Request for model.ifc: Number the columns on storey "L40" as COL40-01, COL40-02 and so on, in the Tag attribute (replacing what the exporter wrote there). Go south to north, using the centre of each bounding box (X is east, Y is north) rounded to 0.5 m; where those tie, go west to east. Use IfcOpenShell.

First a look at what the model holds.

```python
import ifcopenshell
import ifcopenshell.util.element
import ifcopenshell.util.placement

model = ifcopenshell.open("model.ifc")
print(model.schema)
storey = next(s for s in model.by_type("IfcBuildingStorey") if s.Name == "L40")
columns = [e for e in ifcopenshell.util.element.get_decomposition(storey) if e.is_a("IfcColumn")]
for e in sorted(columns, key=lambda e: e.id()):
    origin = ifcopenshell.util.placement.get_local_placement(e.ObjectPlacement)[:3, 3]
    print(e.id(), e.Tag, e.Name, origin.round(2) + 0.0, sep=" | ")
```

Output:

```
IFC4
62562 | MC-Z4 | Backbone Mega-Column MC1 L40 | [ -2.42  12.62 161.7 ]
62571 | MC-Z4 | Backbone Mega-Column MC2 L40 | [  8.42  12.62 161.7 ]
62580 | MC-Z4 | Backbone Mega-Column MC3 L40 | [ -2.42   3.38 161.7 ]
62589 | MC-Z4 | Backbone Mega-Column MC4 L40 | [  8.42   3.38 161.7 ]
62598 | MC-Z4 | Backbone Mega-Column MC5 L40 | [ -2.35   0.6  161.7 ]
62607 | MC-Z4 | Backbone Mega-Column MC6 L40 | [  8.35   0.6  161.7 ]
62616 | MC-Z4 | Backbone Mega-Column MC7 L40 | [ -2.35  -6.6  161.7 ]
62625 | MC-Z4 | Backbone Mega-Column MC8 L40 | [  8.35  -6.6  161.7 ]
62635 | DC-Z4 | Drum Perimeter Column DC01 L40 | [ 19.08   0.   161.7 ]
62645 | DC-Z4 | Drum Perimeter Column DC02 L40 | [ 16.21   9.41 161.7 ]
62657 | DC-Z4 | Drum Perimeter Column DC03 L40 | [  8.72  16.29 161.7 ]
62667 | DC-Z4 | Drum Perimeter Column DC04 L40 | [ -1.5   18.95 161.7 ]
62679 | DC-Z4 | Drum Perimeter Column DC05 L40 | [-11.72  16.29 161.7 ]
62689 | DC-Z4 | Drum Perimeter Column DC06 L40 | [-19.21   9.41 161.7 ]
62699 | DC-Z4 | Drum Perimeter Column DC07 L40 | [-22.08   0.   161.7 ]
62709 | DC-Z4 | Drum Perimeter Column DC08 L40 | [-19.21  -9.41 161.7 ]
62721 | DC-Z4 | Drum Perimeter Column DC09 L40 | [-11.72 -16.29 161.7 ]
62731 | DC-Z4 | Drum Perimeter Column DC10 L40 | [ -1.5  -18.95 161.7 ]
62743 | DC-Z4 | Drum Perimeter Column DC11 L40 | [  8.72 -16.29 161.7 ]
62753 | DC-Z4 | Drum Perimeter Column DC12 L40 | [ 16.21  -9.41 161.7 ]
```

```python
import ifcopenshell
import ifcopenshell.geom
import ifcopenshell.util.element
import ifcopenshell.util.shape

model = ifcopenshell.open("model.ifc")
settings = ifcopenshell.geom.settings()
settings.set("use-world-coords", True)


def centre(element):
    shape = ifcopenshell.geom.create_shape(settings, element)
    return ifcopenshell.util.shape.get_bbox_centroid(shape.geometry)


storey = next(s for s in model.by_type("IfcBuildingStorey") if s.Name == "L40")
columns = [e for e in ifcopenshell.util.element.get_decomposition(storey) if e.is_a("IfcColumn")]

# Insertion points can sit at a corner or the storey origin, so sort by the geometry (in metres).
centres = {e: centre(e) for e in columns}
columns.sort(key=lambda e: (round(centres[e][1] / 0.5), centres[e][0]))

for i, e in enumerate(columns, start=1):
    number = f"COL40-{i:02d}"
    e.Tag = number
    print(e.id(), number)

model.write("model-out.ifc")
```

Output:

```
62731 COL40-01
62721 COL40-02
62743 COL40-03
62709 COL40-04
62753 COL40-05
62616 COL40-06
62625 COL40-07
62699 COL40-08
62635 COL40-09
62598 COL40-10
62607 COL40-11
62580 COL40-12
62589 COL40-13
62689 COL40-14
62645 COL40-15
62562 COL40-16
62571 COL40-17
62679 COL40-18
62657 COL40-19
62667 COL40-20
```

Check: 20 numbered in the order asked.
